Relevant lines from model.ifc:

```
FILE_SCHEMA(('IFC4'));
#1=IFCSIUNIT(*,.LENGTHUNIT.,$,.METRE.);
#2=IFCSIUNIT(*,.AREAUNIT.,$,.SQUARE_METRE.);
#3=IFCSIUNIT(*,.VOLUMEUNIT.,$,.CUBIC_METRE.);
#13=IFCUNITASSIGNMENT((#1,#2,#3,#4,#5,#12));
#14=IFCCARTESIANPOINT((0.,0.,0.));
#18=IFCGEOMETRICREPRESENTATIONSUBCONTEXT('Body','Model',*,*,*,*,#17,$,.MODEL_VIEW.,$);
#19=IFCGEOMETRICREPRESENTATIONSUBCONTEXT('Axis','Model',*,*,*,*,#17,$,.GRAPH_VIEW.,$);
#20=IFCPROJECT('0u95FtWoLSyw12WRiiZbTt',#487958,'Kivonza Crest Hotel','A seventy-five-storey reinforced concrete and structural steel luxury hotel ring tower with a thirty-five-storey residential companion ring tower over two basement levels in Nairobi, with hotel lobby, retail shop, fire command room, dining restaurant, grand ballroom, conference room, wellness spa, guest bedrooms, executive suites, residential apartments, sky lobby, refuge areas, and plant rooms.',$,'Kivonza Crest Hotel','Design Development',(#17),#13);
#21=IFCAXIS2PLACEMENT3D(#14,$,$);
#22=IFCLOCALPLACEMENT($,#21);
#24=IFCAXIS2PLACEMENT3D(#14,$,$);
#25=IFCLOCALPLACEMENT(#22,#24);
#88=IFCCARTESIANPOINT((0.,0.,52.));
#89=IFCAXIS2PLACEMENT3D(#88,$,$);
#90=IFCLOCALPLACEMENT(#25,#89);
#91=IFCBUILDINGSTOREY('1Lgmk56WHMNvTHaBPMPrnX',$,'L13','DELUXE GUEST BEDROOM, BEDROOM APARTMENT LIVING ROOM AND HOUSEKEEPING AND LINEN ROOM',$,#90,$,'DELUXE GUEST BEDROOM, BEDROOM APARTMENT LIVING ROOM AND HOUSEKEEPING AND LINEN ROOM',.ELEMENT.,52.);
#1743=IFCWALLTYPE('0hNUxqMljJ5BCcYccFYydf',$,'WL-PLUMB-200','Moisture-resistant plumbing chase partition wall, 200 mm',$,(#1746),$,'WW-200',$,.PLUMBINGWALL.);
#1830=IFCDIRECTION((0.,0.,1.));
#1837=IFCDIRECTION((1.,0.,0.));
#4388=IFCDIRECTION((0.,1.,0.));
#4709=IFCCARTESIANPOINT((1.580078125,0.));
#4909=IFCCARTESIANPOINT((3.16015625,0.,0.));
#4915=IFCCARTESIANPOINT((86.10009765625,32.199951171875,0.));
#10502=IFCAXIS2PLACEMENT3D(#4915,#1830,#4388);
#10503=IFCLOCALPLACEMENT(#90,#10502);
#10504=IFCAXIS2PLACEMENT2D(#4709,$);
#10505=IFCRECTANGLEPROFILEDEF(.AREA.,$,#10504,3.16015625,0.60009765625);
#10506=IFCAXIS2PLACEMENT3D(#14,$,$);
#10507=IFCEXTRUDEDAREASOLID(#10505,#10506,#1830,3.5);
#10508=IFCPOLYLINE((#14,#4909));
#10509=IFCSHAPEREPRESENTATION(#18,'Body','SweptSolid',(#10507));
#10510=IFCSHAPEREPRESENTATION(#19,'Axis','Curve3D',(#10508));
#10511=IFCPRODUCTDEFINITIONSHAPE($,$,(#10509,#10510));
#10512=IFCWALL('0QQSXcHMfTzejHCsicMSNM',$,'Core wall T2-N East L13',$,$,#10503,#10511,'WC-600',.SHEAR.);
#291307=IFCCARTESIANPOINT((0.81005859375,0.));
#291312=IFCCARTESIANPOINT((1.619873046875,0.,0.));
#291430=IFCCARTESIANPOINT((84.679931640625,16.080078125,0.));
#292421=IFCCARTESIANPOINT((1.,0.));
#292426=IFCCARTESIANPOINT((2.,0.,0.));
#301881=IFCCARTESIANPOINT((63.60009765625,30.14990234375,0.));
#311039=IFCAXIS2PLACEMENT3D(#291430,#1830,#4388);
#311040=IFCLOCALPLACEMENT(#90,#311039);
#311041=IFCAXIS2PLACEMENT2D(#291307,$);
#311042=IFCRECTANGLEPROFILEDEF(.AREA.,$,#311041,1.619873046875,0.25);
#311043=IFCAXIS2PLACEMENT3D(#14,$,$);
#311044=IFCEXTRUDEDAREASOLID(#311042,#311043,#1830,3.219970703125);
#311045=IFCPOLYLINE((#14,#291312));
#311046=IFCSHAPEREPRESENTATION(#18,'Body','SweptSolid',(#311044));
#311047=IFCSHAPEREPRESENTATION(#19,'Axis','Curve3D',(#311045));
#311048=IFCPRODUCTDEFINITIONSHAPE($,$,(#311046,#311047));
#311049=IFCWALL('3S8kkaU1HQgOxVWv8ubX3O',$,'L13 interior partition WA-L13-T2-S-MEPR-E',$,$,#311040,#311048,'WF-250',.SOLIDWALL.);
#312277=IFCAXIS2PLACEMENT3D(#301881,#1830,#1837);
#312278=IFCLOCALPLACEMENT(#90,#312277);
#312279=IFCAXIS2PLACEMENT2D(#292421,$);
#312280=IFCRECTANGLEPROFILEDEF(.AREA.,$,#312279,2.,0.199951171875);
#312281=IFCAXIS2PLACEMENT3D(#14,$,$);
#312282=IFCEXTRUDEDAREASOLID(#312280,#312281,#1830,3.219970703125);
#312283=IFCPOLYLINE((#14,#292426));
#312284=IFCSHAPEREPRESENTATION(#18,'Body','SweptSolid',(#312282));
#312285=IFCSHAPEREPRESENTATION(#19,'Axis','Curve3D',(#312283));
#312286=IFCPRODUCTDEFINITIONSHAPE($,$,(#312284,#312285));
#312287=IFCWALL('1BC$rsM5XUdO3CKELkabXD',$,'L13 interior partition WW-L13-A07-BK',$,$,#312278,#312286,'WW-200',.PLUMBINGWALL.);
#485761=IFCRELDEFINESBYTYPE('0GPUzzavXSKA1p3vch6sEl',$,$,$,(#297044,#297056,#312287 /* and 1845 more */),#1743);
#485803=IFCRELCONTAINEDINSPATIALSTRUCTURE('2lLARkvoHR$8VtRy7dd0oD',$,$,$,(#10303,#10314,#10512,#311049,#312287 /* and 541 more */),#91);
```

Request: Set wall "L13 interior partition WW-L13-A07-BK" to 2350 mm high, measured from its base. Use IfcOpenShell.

```python
import ifcopenshell
import ifcopenshell.geom
import ifcopenshell.util.representation
import ifcopenshell.util.shape
import ifcopenshell.util.unit

model = ifcopenshell.open("model.ifc")
unit_scale = ifcopenshell.util.unit.calculate_unit_scale(model)
settings = ifcopenshell.geom.settings()


def volume(element):
    """Net volume in cubic metres, openings subtracted."""
    shape = ifcopenshell.geom.create_shape(settings, element)
    return ifcopenshell.util.shape.get_volume(shape.geometry)


wall = model.by_guid("1BC$rsM5XUdO3CKELkabXD")
before = volume(wall)

body = ifcopenshell.util.representation.get_representation(wall, "Model", "Body")
solid = body.Items[0]
old_height = solid.Depth
solid.Depth = 2.35 / unit_scale
after = volume(wall)

print(f"height {old_height:g} -> {solid.Depth:g}, volume {before:.3f} -> {after:.3f} m3")

model.write("model_v2.ifc")
```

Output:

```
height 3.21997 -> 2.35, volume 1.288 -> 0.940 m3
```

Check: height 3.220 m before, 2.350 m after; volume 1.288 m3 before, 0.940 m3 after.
